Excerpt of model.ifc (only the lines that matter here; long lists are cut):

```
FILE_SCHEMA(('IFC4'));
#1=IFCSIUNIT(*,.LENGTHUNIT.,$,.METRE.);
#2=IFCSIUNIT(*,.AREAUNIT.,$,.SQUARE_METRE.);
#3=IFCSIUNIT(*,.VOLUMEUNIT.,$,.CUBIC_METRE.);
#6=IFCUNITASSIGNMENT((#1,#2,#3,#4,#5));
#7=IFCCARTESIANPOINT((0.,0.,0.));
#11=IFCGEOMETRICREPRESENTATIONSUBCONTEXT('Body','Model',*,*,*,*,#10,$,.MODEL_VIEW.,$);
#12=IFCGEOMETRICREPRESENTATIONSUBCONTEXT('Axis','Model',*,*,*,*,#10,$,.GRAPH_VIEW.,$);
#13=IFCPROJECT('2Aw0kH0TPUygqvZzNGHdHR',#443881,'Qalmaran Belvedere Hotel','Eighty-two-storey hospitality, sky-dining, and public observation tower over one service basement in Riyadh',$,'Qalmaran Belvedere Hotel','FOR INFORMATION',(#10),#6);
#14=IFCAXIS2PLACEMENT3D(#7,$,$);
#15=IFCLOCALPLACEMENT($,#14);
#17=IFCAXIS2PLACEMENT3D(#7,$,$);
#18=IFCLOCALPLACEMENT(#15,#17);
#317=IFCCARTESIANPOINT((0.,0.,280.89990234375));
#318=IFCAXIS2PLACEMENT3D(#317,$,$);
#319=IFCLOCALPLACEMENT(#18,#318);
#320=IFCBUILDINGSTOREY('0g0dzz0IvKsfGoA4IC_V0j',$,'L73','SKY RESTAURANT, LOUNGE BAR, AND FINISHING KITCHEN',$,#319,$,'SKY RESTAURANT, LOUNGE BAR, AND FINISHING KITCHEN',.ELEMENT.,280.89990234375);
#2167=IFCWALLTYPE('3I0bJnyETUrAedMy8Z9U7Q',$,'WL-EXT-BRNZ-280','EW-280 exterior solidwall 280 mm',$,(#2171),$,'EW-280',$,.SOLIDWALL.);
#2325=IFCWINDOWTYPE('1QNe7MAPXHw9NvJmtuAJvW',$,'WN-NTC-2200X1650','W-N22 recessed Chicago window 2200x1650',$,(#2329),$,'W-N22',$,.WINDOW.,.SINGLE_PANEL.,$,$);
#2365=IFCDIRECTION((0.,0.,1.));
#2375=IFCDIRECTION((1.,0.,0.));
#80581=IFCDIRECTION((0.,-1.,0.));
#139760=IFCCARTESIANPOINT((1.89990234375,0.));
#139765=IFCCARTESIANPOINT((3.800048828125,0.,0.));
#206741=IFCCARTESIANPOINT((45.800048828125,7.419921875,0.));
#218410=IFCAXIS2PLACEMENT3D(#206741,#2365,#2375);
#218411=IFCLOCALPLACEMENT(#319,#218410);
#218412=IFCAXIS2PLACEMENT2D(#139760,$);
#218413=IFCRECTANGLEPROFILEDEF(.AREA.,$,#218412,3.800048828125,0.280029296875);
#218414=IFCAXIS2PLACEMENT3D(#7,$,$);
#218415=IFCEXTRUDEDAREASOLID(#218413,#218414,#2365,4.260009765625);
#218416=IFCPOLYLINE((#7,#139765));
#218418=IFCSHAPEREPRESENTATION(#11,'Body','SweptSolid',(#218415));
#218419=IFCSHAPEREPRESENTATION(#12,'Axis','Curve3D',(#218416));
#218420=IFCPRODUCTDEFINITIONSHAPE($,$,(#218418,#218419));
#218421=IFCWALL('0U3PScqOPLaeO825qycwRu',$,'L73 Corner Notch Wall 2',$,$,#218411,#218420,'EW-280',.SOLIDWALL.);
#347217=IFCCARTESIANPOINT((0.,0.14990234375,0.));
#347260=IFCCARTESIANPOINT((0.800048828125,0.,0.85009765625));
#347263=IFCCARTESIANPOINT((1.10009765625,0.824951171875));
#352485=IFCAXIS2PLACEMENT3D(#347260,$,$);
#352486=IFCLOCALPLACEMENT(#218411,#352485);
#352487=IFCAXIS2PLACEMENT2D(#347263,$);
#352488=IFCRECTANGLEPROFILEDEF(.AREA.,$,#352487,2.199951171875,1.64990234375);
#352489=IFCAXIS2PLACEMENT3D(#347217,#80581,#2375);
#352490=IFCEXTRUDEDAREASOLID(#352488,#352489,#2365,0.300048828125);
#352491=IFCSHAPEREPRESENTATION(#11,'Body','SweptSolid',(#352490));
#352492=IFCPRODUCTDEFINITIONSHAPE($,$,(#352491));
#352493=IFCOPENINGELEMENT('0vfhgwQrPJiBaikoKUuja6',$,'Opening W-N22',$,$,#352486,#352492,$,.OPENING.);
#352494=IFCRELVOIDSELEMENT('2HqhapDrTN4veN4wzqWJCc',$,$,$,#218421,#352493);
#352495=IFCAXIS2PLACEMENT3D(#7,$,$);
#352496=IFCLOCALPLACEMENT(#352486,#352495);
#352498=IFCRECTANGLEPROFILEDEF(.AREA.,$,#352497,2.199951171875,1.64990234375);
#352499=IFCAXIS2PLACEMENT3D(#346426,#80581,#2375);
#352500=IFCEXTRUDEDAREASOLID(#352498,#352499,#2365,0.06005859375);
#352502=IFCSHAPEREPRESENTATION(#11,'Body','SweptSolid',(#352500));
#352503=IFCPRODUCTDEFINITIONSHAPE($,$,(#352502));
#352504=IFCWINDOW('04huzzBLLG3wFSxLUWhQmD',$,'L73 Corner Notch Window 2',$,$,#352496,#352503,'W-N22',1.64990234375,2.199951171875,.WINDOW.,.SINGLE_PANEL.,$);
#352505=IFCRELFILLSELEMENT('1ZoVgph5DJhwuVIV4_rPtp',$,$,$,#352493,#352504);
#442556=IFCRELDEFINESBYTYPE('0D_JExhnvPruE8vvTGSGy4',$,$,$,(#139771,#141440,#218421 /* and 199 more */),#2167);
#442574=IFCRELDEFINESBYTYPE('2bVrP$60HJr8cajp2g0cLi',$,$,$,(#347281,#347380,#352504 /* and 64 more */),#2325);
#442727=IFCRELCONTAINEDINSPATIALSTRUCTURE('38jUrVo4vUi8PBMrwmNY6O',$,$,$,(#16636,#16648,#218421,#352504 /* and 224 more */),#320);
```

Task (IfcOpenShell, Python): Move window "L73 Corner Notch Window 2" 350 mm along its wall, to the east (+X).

```python
import ifcopenshell
import ifcopenshell.api.geometry
import ifcopenshell.util.placement
import ifcopenshell.util.unit

model = ifcopenshell.open("model.ifc")
unit_scale = ifcopenshell.util.unit.calculate_unit_scale(model)

window = model.by_guid("04huzzBLLG3wFSxLUWhQmD")
opening = window.FillsVoids[0].RelatingOpeningElement
wall = opening.VoidsElements[0].RelatingBuildingElement

wall_matrix = ifcopenshell.util.placement.get_local_placement(wall.ObjectPlacement)
shift = wall_matrix[:3, 0] * 0.35 / unit_scale
before = ifcopenshell.util.placement.get_local_placement(window.ObjectPlacement)[:3, 3].copy()

# The window is placed relative to its opening, so it follows when the opening moves.
matrix = ifcopenshell.util.placement.get_local_placement(opening.ObjectPlacement)
matrix[:3, 3] += shift
ifcopenshell.api.geometry.edit_object_placement(
    model, product=opening, matrix=matrix, is_si=False, should_transform_children=True
)

after = ifcopenshell.util.placement.get_local_placement(window.ObjectPlacement)[:3, 3]
print("window moved by", (after - before).round(3) + 0.0)

model.write("model_v2.ifc")
```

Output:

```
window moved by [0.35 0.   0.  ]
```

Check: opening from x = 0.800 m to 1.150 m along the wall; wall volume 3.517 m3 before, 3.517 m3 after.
